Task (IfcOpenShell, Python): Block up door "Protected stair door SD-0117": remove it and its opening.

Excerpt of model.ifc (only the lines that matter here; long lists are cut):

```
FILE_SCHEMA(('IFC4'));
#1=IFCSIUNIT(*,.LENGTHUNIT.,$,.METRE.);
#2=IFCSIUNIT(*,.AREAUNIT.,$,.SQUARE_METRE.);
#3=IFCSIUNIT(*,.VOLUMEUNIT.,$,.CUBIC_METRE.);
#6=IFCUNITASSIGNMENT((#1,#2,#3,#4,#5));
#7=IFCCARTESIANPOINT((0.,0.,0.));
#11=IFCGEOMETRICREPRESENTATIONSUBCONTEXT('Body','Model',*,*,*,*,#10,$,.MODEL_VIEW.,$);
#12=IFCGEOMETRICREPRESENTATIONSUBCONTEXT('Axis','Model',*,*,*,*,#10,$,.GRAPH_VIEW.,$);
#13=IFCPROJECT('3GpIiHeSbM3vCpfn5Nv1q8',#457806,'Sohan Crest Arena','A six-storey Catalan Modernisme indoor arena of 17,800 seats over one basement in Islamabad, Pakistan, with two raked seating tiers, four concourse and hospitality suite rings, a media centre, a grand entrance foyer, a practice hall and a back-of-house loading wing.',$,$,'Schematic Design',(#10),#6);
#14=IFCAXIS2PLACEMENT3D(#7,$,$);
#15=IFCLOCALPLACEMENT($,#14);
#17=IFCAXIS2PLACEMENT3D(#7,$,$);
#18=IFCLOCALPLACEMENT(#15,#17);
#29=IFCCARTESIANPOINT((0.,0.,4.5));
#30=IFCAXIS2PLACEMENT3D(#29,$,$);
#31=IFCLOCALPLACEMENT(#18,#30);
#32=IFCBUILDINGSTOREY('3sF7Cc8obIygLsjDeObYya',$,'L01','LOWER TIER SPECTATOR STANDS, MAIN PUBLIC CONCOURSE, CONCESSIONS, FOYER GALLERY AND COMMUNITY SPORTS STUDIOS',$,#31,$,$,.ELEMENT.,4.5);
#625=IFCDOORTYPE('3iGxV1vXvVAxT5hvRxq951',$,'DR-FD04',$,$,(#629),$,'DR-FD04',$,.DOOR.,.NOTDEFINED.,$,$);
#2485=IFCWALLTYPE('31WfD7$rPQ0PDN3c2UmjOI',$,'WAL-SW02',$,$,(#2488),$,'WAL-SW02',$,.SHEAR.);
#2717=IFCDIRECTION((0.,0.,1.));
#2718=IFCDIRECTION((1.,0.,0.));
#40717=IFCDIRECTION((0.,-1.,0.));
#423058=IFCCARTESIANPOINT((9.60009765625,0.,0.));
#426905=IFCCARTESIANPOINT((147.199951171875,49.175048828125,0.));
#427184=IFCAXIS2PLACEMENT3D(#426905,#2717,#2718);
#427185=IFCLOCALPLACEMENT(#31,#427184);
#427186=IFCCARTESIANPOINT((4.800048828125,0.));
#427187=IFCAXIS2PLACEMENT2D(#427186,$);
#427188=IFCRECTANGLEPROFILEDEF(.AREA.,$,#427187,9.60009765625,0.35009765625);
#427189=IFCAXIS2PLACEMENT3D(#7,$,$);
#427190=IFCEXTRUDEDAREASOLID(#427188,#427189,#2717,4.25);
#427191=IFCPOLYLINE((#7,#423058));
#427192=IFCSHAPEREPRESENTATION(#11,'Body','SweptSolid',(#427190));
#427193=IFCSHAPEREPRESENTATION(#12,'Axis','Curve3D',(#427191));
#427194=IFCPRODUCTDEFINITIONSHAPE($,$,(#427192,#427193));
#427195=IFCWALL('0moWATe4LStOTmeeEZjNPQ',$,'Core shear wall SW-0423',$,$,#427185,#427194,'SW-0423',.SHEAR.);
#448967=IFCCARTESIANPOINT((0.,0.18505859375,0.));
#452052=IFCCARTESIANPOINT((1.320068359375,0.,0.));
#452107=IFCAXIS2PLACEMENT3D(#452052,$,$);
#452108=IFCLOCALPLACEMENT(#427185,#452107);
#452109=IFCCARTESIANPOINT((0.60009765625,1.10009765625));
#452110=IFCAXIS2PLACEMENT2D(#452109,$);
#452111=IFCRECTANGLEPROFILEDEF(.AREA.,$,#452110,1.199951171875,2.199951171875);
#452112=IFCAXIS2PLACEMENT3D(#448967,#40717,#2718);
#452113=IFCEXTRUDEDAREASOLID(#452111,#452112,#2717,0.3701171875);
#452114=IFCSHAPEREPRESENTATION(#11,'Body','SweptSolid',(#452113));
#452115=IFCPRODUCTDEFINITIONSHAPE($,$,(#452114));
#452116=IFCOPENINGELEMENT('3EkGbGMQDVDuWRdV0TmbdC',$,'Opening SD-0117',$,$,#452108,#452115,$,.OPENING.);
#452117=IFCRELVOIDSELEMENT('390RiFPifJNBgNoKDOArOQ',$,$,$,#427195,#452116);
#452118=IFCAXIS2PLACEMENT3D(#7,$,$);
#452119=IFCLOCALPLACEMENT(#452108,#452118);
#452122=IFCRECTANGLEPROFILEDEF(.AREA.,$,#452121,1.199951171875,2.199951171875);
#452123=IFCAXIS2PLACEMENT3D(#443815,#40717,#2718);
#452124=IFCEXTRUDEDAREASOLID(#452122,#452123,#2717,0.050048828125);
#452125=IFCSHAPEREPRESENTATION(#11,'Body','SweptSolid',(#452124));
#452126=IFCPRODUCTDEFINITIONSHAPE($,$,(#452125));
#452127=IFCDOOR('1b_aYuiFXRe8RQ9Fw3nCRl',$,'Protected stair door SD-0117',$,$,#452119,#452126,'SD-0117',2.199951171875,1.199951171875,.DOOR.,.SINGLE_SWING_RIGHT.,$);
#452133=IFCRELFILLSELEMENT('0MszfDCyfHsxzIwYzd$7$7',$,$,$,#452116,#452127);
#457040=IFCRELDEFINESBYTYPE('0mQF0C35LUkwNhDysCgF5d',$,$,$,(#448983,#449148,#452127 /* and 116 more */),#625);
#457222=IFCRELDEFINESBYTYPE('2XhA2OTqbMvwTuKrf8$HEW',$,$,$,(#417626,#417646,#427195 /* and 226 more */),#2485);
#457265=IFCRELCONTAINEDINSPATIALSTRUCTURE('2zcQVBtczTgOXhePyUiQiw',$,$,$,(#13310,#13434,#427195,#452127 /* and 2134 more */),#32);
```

```python
import ifcopenshell
import ifcopenshell.api.feature
import ifcopenshell.api.root
import ifcopenshell.geom
import ifcopenshell.util.shape

model = ifcopenshell.open("model.ifc")
settings = ifcopenshell.geom.settings()


def volume(element):
    """Net volume in cubic metres, openings subtracted."""
    shape = ifcopenshell.geom.create_shape(settings, element)
    return ifcopenshell.util.shape.get_volume(shape.geometry)


door = model.by_id(452127)
opening = door.FillsVoids[0].RelatingOpeningElement
wall = opening.VoidsElements[0].RelatingBuildingElement
before = volume(wall)

ifcopenshell.api.root.remove_product(model, product=door)
ifcopenshell.api.feature.remove_feature(model, feature=opening)

after = volume(wall)

print(f"wall volume {before:.3f} -> {after:.3f} m3")

model.write("model_edited.ifc")
```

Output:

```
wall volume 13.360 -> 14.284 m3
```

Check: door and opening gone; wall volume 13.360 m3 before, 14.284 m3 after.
